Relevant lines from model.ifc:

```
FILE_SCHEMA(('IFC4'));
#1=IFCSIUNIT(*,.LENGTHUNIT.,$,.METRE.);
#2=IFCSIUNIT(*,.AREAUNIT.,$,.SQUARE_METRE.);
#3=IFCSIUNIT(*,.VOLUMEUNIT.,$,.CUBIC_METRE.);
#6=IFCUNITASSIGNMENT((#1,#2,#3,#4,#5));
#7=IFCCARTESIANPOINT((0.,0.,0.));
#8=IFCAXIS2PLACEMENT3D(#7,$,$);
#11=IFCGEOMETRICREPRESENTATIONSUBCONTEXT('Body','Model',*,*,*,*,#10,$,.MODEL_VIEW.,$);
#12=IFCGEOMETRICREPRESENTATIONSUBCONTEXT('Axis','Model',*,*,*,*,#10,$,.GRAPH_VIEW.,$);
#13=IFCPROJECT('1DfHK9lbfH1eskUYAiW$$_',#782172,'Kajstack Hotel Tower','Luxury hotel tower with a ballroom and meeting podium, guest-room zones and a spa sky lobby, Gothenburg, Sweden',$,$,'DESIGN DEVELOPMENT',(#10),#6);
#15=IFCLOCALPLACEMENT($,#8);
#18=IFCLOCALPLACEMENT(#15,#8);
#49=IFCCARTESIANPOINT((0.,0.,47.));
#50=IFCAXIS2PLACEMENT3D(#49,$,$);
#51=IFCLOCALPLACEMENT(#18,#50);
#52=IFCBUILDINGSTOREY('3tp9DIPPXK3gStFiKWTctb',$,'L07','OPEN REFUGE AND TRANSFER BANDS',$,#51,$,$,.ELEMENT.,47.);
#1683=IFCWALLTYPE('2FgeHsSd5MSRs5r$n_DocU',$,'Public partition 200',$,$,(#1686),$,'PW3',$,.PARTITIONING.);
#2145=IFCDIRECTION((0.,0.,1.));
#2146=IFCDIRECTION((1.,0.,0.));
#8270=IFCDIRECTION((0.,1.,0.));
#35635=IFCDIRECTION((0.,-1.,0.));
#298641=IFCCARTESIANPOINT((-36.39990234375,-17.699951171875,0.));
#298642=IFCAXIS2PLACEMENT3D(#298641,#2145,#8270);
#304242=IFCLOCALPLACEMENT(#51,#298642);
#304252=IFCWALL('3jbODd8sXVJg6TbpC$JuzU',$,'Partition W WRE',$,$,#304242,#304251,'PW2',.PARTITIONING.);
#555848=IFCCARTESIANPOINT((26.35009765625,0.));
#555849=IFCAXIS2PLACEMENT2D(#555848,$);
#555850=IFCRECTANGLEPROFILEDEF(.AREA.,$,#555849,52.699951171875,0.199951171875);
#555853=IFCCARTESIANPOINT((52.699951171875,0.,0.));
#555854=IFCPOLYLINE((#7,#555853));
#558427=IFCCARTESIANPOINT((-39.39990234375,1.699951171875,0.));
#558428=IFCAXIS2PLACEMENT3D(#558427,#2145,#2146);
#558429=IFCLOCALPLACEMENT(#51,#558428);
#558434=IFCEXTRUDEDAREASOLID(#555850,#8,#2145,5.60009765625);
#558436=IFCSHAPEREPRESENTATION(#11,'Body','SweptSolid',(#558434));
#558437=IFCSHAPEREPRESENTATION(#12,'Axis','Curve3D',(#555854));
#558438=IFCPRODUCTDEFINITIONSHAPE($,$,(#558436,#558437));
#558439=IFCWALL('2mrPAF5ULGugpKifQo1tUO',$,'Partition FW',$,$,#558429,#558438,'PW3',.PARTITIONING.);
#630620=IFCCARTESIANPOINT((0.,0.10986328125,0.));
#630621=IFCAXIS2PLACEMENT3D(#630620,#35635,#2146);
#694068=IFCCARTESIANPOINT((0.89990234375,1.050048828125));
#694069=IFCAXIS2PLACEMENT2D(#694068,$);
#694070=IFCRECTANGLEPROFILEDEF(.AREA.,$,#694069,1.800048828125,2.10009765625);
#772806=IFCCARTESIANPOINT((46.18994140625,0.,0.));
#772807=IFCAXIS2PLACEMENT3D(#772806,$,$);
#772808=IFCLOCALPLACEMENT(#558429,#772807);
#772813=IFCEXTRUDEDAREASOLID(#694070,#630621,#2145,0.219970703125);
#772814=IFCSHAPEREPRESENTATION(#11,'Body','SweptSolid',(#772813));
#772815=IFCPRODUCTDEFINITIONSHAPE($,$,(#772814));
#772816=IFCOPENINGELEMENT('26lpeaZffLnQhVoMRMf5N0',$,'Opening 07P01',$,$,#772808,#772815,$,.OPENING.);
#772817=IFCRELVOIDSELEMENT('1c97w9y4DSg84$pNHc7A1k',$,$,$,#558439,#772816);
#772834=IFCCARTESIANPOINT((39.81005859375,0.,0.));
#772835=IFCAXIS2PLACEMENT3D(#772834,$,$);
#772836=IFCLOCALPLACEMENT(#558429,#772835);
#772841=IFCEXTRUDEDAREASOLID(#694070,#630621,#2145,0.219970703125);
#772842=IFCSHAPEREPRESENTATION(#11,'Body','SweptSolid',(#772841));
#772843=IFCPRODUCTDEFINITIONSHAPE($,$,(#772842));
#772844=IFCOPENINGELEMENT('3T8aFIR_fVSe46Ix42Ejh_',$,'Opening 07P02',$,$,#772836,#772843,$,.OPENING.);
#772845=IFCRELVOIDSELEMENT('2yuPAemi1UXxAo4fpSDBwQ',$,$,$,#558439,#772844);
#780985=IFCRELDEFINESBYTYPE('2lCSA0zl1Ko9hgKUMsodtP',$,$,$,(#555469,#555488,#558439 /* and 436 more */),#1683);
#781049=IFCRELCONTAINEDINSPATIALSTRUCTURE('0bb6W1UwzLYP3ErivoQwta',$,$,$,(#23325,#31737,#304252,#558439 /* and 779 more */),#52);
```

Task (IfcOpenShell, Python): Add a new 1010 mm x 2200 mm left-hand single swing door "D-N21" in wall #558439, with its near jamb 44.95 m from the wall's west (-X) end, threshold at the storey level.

```python
import numpy as np
import ifcopenshell
import ifcopenshell.api.feature
import ifcopenshell.api.geometry
import ifcopenshell.api.root
import ifcopenshell.api.spatial
import ifcopenshell.geom
import ifcopenshell.util.element
import ifcopenshell.util.placement
import ifcopenshell.util.representation
import ifcopenshell.util.shape
import ifcopenshell.util.unit

model = ifcopenshell.open("model.ifc")
unit_scale = ifcopenshell.util.unit.calculate_unit_scale(model)
settings = ifcopenshell.geom.settings()


def volume(element):
    """Net volume in cubic metres, openings subtracted."""
    shape = ifcopenshell.geom.create_shape(settings, element)
    return ifcopenshell.util.shape.get_volume(shape.geometry)


wall = model.by_guid("2mrPAF5ULGugpKifQo1tUO")
storey = ifcopenshell.util.element.get_container(wall, ifc_class="IfcBuildingStorey")
context = ifcopenshell.util.representation.get_context(model, "Model", "Body", "MODEL_VIEW")
before = volume(wall)

width, height, from_end, sill = 1.01, 2.2, 44.95, 0.0  # metres

# The wall runs along its own X axis, and the end named is its -X end.
wall_shape = ifcopenshell.geom.create_shape(settings, wall)
x, y, z = ifcopenshell.util.shape.get_vertices(wall_shape.geometry).T
start = x.min() + from_end
face, thickness = float(y.min()), float(y.max() - y.min())
wall_matrix = ifcopenshell.util.placement.get_local_placement(wall.ObjectPlacement)
level = ifcopenshell.util.placement.get_local_placement(storey.ObjectPlacement)[2, 3]


def in_wall(x, y):
    """Placement at x, y metres in the wall's axes, at sill height."""
    matrix = wall_matrix.copy()
    matrix[:, 3] = wall_matrix @ np.array([x / unit_scale, y / unit_scale, 0.0, 1.0])
    matrix[2, 3] = level + sill / unit_scale
    return matrix


# Opening: a box that overshoots both wall faces by 50 mm.
opening = ifcopenshell.api.root.create_entity(model, ifc_class="IfcOpeningElement", predefined_type="OPENING")
box = ifcopenshell.api.geometry.add_wall_representation(
    model, context=context, length=width, height=height, thickness=thickness + 0.1
)
ifcopenshell.api.geometry.assign_representation(model, product=opening, representation=box)
ifcopenshell.api.geometry.edit_object_placement(model, product=opening, matrix=in_wall(start, face - 0.05), is_si=False)
ifcopenshell.api.feature.add_feature(model, feature=opening, element=wall)

door = ifcopenshell.api.root.create_entity(model, ifc_class="IfcDoor", name="D-N21", predefined_type="DOOR")
door.OverallWidth, door.OverallHeight = width / unit_scale, height / unit_scale
door.OperationType = "SINGLE_SWING_LEFT"
body = ifcopenshell.api.geometry.add_door_representation(
    model,
    context=context,
    overall_width=door.OverallWidth,
    overall_height=door.OverallHeight,
    operation_type="SINGLE_SWING_LEFT",
    lining_properties={"LiningDepth": thickness / unit_scale, "ThresholdDepth": thickness / unit_scale},
)
ifcopenshell.api.geometry.assign_representation(model, product=door, representation=body)
ifcopenshell.api.spatial.assign_container(model, products=[door], relating_structure=storey)
ifcopenshell.api.feature.add_filling(model, opening=opening, element=door)

# The lining spans the wall, so the door starts at the wall face.
ifcopenshell.api.geometry.edit_object_placement(model, product=door, matrix=in_wall(start, face), is_si=False)

after = volume(wall)

print(f"wall volume {before:.3f} -> {after:.3f} m3")

model.write("model_v2.ifc")
```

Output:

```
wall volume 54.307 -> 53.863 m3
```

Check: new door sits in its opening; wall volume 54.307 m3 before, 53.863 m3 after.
